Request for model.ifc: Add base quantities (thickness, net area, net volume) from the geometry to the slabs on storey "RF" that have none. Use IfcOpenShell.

First a look at what the model holds.

```python
import ifcopenshell
import ifcopenshell.util.element
import ifcopenshell.util.unit

model = ifcopenshell.open("model.ifc")
print(model.schema)
for unit_type in ("LENGTHUNIT", "AREAUNIT", "VOLUMEUNIT"):
    print(unit_type, ifcopenshell.util.unit.calculate_unit_scale(model, unit_type))
storey = next(s for s in model.by_type("IfcBuildingStorey") if s.Name == "RF")
slabs = [e for e in ifcopenshell.util.element.get_decomposition(storey) if e.is_a("IfcSlab")]
for e in sorted(slabs, key=lambda e: e.id()):
    print(e.id(), e.is_a(), e.Name, list(ifcopenshell.util.element.get_psets(e, qtos_only=True)), sep=" | ")
```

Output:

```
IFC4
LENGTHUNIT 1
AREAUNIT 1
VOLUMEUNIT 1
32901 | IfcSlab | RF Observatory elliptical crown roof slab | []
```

```python
import ifcopenshell
import ifcopenshell.api.pset
import ifcopenshell.geom
import ifcopenshell.util.element
import ifcopenshell.util.shape
import ifcopenshell.util.unit

model = ifcopenshell.open("model.ifc")
unit_scale = ifcopenshell.util.unit.calculate_unit_scale(model)
area_scale = ifcopenshell.util.unit.calculate_unit_scale(model, "AREAUNIT")
volume_scale = ifcopenshell.util.unit.calculate_unit_scale(model, "VOLUMEUNIT")
settings = ifcopenshell.geom.settings()

storey = next(s for s in model.by_type("IfcBuildingStorey") if s.Name == "RF")
slabs = [e for e in ifcopenshell.util.element.get_decomposition(storey) if e.is_a("IfcSlab")]

for e in sorted(slabs, key=lambda e: e.id()):
    if ifcopenshell.util.element.get_psets(e, qtos_only=True, should_inherit=False):
        continue
    # Geometry comes back in metres, in the element's own axes.
    shape = ifcopenshell.geom.create_shape(settings, e)
    values = {
        "Width": ifcopenshell.util.shape.get_z(shape.geometry) / unit_scale,
        "NetArea": ifcopenshell.util.shape.get_footprint_area(shape.geometry) / area_scale,
        "NetVolume": ifcopenshell.util.shape.get_volume(shape.geometry) / volume_scale,
    }
    qto = ifcopenshell.api.pset.add_qto(model, product=e, name="Qto_SlabBaseQuantities")
    ifcopenshell.api.pset.edit_qto(model, qto=qto, properties=values)
    print(e.id(), {k: round(v, 3) for k, v in values.items()})

model.write("model_rev.ifc")
```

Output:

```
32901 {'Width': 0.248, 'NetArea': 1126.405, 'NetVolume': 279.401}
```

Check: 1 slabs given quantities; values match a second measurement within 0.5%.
